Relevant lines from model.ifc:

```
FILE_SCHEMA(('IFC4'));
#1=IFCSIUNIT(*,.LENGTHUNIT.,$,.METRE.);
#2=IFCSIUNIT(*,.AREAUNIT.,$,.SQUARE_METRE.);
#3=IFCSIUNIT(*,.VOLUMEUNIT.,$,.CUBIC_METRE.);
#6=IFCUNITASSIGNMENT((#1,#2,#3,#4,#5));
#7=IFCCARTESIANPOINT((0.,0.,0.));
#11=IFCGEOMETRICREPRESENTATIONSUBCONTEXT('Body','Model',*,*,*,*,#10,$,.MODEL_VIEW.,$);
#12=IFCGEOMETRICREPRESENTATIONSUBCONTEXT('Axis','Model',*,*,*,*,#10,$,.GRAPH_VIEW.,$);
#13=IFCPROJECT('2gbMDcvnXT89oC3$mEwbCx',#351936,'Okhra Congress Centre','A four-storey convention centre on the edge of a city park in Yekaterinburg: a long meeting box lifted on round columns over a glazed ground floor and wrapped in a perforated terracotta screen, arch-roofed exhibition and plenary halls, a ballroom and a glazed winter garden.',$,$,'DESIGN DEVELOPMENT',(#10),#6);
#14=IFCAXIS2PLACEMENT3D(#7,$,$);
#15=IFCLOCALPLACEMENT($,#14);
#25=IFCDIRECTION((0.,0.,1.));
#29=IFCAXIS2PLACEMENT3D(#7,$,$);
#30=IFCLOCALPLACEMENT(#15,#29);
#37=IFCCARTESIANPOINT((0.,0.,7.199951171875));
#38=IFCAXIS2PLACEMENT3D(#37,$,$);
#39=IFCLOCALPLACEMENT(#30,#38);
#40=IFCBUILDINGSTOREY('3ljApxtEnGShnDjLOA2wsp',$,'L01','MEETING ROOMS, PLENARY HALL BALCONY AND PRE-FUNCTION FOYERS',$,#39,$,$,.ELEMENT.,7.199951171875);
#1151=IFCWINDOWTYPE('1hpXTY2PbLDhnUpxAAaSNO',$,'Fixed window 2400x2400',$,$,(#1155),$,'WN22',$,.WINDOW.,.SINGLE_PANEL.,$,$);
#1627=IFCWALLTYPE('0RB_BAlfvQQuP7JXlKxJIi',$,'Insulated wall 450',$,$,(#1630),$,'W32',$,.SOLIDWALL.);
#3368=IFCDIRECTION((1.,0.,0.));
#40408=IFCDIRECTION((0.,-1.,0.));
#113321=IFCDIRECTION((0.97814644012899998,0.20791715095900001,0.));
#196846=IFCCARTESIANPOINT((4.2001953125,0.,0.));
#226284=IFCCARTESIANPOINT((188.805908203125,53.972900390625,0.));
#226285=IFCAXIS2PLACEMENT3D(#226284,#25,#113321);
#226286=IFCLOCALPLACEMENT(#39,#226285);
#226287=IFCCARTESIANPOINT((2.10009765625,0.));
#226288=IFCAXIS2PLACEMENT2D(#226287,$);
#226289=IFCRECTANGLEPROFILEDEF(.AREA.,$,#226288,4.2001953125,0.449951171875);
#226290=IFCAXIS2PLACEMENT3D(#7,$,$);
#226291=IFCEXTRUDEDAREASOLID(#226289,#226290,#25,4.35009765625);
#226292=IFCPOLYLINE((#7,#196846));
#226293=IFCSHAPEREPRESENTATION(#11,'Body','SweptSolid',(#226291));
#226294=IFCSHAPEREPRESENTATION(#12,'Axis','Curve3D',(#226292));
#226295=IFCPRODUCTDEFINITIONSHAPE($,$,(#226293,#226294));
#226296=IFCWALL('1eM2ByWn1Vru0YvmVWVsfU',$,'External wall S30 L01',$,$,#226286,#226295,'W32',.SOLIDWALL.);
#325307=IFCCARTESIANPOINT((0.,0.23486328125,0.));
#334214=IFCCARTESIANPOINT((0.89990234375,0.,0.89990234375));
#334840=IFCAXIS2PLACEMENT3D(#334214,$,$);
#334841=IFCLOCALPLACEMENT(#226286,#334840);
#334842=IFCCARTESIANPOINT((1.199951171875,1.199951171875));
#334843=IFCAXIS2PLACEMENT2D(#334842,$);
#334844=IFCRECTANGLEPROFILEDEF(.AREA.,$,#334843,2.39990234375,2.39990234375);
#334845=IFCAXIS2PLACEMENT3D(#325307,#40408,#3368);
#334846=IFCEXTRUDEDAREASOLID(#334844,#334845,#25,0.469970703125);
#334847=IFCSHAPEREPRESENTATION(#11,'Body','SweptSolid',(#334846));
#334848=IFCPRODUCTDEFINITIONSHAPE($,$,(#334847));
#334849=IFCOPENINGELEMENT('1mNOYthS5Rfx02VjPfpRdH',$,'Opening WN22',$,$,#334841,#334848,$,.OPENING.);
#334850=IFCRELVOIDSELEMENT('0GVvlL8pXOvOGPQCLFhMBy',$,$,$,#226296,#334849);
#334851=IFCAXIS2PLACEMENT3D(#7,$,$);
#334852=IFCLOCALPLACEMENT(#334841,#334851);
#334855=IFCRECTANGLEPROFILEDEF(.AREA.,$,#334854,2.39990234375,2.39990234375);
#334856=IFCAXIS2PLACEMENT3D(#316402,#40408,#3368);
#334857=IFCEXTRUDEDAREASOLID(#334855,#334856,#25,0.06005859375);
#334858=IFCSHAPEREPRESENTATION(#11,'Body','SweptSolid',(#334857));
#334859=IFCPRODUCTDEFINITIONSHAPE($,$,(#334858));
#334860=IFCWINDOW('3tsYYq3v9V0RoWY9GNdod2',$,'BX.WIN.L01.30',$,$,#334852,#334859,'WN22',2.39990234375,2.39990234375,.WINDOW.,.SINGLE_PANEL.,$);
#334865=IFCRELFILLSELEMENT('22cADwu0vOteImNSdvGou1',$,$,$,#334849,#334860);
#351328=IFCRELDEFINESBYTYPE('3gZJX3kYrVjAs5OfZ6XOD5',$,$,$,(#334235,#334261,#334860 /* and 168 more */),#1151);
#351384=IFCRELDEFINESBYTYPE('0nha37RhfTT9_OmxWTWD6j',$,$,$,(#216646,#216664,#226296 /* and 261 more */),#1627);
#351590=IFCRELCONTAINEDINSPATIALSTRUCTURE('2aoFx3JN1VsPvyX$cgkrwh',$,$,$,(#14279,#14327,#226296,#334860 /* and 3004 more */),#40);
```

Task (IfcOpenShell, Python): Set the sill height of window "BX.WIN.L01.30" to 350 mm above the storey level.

```python
import numpy as np
import ifcopenshell
import ifcopenshell.api.geometry
import ifcopenshell.geom
import ifcopenshell.util.element
import ifcopenshell.util.placement
import ifcopenshell.util.shape
import ifcopenshell.util.unit

model = ifcopenshell.open("model.ifc")
unit_scale = ifcopenshell.util.unit.calculate_unit_scale(model)

window = model.by_guid("3tsYYq3v9V0RoWY9GNdod2")
opening = window.FillsVoids[0].RelatingOpeningElement
storey = ifcopenshell.util.element.get_container(window, ifc_class="IfcBuildingStorey")
level = ifcopenshell.util.placement.get_local_placement(storey.ObjectPlacement)[2, 3]

# The opening's origin need not be at the sill, so measure its lowest point.
shape = ifcopenshell.geom.create_shape(ifcopenshell.geom.settings(), opening)
bottom = ifcopenshell.util.shape.get_shape_bottom_elevation(shape, shape.geometry) / unit_scale
dz = level + 0.35 - bottom

shift = np.array([0.0, 0.0, dz])
# The window is placed relative to its opening, so it follows when the opening moves.
matrix = ifcopenshell.util.placement.get_local_placement(opening.ObjectPlacement)
matrix[:3, 3] += shift
ifcopenshell.api.geometry.edit_object_placement(
    model, product=opening, matrix=matrix, is_si=False, should_transform_children=True
)

print(f"moved by {dz * unit_scale:+.3f} m")

model.write("model_edited.ifc")
```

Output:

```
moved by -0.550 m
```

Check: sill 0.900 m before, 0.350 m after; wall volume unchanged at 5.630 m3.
